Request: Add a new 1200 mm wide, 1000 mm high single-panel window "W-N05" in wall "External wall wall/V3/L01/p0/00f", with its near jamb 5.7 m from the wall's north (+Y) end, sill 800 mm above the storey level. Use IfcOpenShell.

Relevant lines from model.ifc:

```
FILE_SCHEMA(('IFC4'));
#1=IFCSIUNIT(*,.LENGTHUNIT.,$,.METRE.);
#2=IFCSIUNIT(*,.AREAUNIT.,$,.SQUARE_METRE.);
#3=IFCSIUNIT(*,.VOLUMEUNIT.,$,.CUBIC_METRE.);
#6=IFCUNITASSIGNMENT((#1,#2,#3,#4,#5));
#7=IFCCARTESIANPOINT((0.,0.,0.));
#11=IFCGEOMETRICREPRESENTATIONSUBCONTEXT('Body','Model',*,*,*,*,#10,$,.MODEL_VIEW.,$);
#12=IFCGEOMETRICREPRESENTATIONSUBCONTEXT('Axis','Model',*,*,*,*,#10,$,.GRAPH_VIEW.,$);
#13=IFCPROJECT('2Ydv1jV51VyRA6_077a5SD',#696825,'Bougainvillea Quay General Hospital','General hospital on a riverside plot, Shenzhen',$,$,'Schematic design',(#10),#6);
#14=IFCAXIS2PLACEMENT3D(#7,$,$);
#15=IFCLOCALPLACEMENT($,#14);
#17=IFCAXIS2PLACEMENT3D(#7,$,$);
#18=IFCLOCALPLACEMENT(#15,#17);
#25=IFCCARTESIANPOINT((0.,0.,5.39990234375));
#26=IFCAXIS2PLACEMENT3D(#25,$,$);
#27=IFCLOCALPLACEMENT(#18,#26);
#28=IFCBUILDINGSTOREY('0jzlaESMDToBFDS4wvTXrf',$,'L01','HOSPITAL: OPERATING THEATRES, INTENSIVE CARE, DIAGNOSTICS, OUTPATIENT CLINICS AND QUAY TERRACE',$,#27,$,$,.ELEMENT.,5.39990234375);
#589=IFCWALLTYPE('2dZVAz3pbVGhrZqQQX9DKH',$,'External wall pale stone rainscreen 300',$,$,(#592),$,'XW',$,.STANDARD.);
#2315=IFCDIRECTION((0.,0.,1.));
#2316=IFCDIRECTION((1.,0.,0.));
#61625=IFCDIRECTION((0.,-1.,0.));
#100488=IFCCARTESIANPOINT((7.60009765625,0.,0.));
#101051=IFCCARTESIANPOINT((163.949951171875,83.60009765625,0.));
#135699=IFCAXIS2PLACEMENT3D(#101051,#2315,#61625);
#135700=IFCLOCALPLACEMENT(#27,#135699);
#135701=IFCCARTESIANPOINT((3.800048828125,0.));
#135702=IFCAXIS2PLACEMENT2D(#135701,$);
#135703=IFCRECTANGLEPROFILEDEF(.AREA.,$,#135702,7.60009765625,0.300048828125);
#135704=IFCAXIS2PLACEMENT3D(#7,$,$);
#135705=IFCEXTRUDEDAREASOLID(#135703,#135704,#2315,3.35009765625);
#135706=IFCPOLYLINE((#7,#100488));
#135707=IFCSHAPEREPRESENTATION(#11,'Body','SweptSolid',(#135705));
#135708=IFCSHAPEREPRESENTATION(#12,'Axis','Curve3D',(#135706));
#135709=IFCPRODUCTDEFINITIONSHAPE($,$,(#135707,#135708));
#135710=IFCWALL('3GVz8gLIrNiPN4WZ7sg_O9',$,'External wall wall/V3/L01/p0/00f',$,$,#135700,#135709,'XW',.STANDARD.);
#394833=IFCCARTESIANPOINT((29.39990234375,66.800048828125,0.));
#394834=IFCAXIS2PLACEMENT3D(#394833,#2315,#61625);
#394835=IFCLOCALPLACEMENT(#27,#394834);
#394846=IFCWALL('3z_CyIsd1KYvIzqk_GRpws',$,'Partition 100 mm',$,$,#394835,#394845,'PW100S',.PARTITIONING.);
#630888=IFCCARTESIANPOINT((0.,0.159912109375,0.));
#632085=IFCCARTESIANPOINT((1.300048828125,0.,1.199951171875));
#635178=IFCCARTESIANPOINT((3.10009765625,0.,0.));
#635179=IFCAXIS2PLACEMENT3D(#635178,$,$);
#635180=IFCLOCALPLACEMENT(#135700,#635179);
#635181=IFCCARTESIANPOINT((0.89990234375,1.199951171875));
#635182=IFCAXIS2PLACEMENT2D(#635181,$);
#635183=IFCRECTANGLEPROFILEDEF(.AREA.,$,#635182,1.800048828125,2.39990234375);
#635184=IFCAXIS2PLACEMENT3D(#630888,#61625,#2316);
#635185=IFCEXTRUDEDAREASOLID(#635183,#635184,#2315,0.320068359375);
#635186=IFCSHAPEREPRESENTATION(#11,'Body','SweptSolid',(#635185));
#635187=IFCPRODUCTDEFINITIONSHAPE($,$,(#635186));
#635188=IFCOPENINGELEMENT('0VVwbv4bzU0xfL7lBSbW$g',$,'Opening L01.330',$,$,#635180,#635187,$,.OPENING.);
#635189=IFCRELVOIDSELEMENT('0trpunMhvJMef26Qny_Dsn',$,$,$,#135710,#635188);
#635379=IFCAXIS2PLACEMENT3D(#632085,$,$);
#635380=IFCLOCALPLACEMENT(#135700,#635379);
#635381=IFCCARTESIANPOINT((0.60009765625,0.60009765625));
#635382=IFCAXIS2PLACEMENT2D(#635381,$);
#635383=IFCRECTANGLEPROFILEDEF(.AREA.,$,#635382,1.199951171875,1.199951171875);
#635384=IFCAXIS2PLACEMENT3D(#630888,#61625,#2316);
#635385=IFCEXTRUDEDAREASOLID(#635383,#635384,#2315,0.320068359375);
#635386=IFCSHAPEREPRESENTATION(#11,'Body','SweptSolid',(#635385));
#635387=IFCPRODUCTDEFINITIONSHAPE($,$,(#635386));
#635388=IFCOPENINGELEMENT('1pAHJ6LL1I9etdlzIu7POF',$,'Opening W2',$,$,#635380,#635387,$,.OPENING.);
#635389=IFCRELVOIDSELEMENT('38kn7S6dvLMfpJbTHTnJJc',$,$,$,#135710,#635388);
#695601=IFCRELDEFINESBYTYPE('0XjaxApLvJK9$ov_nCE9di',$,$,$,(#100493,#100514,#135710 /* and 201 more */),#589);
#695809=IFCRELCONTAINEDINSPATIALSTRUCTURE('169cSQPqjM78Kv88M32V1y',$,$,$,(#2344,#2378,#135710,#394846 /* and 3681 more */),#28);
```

```python
import numpy as np
import ifcopenshell
import ifcopenshell.api.feature
import ifcopenshell.api.geometry
import ifcopenshell.api.root
import ifcopenshell.api.spatial
import ifcopenshell.geom
import ifcopenshell.util.element
import ifcopenshell.util.placement
import ifcopenshell.util.representation
import ifcopenshell.util.shape
import ifcopenshell.util.unit

model = ifcopenshell.open("model.ifc")
unit_scale = ifcopenshell.util.unit.calculate_unit_scale(model)
settings = ifcopenshell.geom.settings()


def volume(element):
    """Net volume in cubic metres, openings subtracted."""
    shape = ifcopenshell.geom.create_shape(settings, element)
    return ifcopenshell.util.shape.get_volume(shape.geometry)


wall = model.by_id(135710)
storey = ifcopenshell.util.element.get_container(wall, ifc_class="IfcBuildingStorey")
context = ifcopenshell.util.representation.get_context(model, "Model", "Body", "MODEL_VIEW")
before = volume(wall)

width, height, from_end, sill = 1.2, 1, 5.7, 0.8  # metres

# The wall runs along its own X axis, and the end named is its -X end.
wall_shape = ifcopenshell.geom.create_shape(settings, wall)
x, y, z = ifcopenshell.util.shape.get_vertices(wall_shape.geometry).T
start = x.min() + from_end
face, thickness = float(y.min()), float(y.max() - y.min())
wall_matrix = ifcopenshell.util.placement.get_local_placement(wall.ObjectPlacement)
level = ifcopenshell.util.placement.get_local_placement(storey.ObjectPlacement)[2, 3]


def in_wall(x, y):
    """Placement at x, y metres in the wall's axes, at sill height."""
    matrix = wall_matrix.copy()
    matrix[:, 3] = wall_matrix @ np.array([x / unit_scale, y / unit_scale, 0.0, 1.0])
    matrix[2, 3] = level + sill / unit_scale
    return matrix


# Opening: a box that overshoots both wall faces by 50 mm.
opening = ifcopenshell.api.root.create_entity(model, ifc_class="IfcOpeningElement", predefined_type="OPENING")
box = ifcopenshell.api.geometry.add_wall_representation(
    model, context=context, length=width, height=height, thickness=thickness + 0.1
)
ifcopenshell.api.geometry.assign_representation(model, product=opening, representation=box)
ifcopenshell.api.geometry.edit_object_placement(model, product=opening, matrix=in_wall(start, face - 0.05), is_si=False)
ifcopenshell.api.feature.add_feature(model, feature=opening, element=wall)

window = ifcopenshell.api.root.create_entity(model, ifc_class="IfcWindow", name="W-N05", predefined_type="WINDOW")
window.OverallWidth, window.OverallHeight = width / unit_scale, height / unit_scale
window.PartitioningType = "SINGLE_PANEL"
body = ifcopenshell.api.geometry.add_window_representation(
    model,
    context=context,
    overall_width=window.OverallWidth,
    overall_height=window.OverallHeight,
    partition_type="SINGLE_PANEL",
)
ifcopenshell.api.geometry.assign_representation(model, product=window, representation=body)
ifcopenshell.api.spatial.assign_container(model, products=[window], relating_structure=storey)
ifcopenshell.api.feature.add_filling(model, opening=opening, element=window)

# Centre the window in the wall's thickness.
ifcopenshell.api.geometry.edit_object_placement(model, product=window, matrix=in_wall(start, face), is_si=False)
window_shape = ifcopenshell.geom.create_shape(settings, window)
depth = ifcopenshell.util.shape.get_vertices(window_shape.geometry)[:, 1]
offset = face + thickness / 2 - (depth.min() + depth.max()) / 2
ifcopenshell.api.geometry.edit_object_placement(model, product=window, matrix=in_wall(start, offset), is_si=False)

after = volume(wall)

print(f"wall volume {before:.3f} -> {after:.3f} m3")

model.write("model_edited.ifc")
```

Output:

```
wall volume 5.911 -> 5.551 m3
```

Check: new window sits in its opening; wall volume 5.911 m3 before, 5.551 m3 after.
